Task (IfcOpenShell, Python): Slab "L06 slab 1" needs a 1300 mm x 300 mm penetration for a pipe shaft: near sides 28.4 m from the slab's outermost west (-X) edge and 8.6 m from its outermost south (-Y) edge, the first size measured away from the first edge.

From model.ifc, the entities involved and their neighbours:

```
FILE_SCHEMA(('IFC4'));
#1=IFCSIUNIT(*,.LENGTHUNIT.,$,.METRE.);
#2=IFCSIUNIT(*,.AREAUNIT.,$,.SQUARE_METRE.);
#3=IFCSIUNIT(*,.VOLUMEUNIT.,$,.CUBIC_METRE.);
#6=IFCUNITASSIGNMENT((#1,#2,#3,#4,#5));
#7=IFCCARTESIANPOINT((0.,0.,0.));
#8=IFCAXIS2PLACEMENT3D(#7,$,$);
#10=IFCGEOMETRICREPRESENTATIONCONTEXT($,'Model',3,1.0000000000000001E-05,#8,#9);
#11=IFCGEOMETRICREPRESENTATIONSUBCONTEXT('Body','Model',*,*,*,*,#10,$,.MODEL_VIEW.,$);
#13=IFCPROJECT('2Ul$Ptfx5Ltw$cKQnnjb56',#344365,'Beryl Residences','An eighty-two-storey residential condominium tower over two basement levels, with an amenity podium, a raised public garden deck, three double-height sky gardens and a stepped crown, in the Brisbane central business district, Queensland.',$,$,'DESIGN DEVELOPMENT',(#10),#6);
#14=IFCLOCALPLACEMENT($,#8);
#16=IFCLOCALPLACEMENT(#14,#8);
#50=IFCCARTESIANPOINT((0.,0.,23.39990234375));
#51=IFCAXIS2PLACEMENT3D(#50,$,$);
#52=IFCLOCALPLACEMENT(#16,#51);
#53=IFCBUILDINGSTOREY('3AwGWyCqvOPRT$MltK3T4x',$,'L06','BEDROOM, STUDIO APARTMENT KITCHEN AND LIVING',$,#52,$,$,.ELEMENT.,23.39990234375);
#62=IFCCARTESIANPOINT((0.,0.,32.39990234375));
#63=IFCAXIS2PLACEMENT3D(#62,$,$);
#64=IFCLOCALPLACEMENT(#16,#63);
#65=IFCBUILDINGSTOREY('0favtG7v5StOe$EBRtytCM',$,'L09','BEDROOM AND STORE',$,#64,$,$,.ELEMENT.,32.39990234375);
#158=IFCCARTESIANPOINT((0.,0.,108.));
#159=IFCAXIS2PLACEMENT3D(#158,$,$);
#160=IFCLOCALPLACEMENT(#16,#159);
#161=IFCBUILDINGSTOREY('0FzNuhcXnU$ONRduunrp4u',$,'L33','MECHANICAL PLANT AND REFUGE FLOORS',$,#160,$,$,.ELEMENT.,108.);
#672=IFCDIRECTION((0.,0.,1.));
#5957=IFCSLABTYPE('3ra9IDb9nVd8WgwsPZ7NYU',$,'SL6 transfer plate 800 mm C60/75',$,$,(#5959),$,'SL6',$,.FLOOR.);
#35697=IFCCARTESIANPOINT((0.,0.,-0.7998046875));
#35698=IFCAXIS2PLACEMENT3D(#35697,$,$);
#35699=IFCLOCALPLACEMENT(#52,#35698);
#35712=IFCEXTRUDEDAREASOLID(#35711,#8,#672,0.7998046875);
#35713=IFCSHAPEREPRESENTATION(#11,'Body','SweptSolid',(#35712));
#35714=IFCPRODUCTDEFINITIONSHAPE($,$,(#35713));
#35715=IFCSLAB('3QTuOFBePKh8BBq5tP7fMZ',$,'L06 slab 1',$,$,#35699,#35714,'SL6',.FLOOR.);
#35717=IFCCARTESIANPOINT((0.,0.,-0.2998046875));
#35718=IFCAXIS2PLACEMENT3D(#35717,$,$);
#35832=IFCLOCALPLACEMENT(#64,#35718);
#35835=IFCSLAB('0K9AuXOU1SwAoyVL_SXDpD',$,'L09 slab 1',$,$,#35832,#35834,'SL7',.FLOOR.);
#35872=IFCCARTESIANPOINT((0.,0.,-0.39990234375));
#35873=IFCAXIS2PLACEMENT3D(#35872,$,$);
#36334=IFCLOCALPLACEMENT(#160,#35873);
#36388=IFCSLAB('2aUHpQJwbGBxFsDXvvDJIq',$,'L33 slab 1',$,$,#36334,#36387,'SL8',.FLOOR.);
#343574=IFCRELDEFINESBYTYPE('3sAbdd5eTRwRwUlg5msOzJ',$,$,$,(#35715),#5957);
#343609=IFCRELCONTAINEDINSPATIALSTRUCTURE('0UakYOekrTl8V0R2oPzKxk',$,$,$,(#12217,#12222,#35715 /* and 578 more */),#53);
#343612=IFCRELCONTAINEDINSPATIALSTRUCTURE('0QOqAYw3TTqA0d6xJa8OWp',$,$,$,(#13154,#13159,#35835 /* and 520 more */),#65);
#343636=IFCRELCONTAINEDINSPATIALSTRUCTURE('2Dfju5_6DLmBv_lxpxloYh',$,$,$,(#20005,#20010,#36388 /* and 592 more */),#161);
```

```python
import numpy as np
import ifcopenshell
import ifcopenshell.api.feature
import ifcopenshell.api.geometry
import ifcopenshell.api.root
import ifcopenshell.geom
import ifcopenshell.util.placement
import ifcopenshell.util.representation
import ifcopenshell.util.shape
import ifcopenshell.util.unit

model = ifcopenshell.open("model.ifc")
unit_scale = ifcopenshell.util.unit.calculate_unit_scale(model)
settings = ifcopenshell.geom.settings()


def volume(element):
    """Net volume in cubic metres, openings subtracted."""
    shape = ifcopenshell.geom.create_shape(settings, element)
    return ifcopenshell.util.shape.get_volume(shape.geometry)


slab = model.by_guid("3QTuOFBePKh8BBq5tP7fMZ")
before = volume(slab)

# Extent in the slab's own axes, in metres. The edges named are its -X and -Y sides.
slab_shape = ifcopenshell.geom.create_shape(settings, slab)
vertices = ifcopenshell.util.shape.get_vertices(slab_shape.geometry)
x_min, y_min, bottom = vertices.min(axis=0)
top = vertices[:, 2].max()

opening = ifcopenshell.api.root.create_entity(model, ifc_class="IfcOpeningElement", name="Pipe shaft opening", predefined_type="OPENING")
context = ifcopenshell.util.representation.get_context(model, "Model", "Body", "MODEL_VIEW")
width, depth = 1.3, 0.3
outline = [(0.0, 0.0), (width, 0.0), (width, depth), (0.0, depth), (0.0, 0.0)]
# Overshoot both faces by 50 mm so the cut is clean.
shape = ifcopenshell.api.geometry.add_slab_representation(
    model, context=context, depth=top - bottom + 0.1, polyline=outline
)
ifcopenshell.api.geometry.assign_representation(model, product=opening, representation=shape)

matrix = ifcopenshell.util.placement.get_local_placement(slab.ObjectPlacement)
matrix[:, 3] = matrix @ np.append(np.array([x_min + 28.4, y_min + 8.6, bottom - 0.05]) / unit_scale, 1.0)
ifcopenshell.api.geometry.edit_object_placement(model, product=opening, matrix=matrix, is_si=False)
ifcopenshell.api.feature.add_feature(model, feature=opening, element=slab)

after = volume(slab)

print(f"slab volume {before:.3f} -> {after:.3f} m3")

model.write("model_rev.ifc")
```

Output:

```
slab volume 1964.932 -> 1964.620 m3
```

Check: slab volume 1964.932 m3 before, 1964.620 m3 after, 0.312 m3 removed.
